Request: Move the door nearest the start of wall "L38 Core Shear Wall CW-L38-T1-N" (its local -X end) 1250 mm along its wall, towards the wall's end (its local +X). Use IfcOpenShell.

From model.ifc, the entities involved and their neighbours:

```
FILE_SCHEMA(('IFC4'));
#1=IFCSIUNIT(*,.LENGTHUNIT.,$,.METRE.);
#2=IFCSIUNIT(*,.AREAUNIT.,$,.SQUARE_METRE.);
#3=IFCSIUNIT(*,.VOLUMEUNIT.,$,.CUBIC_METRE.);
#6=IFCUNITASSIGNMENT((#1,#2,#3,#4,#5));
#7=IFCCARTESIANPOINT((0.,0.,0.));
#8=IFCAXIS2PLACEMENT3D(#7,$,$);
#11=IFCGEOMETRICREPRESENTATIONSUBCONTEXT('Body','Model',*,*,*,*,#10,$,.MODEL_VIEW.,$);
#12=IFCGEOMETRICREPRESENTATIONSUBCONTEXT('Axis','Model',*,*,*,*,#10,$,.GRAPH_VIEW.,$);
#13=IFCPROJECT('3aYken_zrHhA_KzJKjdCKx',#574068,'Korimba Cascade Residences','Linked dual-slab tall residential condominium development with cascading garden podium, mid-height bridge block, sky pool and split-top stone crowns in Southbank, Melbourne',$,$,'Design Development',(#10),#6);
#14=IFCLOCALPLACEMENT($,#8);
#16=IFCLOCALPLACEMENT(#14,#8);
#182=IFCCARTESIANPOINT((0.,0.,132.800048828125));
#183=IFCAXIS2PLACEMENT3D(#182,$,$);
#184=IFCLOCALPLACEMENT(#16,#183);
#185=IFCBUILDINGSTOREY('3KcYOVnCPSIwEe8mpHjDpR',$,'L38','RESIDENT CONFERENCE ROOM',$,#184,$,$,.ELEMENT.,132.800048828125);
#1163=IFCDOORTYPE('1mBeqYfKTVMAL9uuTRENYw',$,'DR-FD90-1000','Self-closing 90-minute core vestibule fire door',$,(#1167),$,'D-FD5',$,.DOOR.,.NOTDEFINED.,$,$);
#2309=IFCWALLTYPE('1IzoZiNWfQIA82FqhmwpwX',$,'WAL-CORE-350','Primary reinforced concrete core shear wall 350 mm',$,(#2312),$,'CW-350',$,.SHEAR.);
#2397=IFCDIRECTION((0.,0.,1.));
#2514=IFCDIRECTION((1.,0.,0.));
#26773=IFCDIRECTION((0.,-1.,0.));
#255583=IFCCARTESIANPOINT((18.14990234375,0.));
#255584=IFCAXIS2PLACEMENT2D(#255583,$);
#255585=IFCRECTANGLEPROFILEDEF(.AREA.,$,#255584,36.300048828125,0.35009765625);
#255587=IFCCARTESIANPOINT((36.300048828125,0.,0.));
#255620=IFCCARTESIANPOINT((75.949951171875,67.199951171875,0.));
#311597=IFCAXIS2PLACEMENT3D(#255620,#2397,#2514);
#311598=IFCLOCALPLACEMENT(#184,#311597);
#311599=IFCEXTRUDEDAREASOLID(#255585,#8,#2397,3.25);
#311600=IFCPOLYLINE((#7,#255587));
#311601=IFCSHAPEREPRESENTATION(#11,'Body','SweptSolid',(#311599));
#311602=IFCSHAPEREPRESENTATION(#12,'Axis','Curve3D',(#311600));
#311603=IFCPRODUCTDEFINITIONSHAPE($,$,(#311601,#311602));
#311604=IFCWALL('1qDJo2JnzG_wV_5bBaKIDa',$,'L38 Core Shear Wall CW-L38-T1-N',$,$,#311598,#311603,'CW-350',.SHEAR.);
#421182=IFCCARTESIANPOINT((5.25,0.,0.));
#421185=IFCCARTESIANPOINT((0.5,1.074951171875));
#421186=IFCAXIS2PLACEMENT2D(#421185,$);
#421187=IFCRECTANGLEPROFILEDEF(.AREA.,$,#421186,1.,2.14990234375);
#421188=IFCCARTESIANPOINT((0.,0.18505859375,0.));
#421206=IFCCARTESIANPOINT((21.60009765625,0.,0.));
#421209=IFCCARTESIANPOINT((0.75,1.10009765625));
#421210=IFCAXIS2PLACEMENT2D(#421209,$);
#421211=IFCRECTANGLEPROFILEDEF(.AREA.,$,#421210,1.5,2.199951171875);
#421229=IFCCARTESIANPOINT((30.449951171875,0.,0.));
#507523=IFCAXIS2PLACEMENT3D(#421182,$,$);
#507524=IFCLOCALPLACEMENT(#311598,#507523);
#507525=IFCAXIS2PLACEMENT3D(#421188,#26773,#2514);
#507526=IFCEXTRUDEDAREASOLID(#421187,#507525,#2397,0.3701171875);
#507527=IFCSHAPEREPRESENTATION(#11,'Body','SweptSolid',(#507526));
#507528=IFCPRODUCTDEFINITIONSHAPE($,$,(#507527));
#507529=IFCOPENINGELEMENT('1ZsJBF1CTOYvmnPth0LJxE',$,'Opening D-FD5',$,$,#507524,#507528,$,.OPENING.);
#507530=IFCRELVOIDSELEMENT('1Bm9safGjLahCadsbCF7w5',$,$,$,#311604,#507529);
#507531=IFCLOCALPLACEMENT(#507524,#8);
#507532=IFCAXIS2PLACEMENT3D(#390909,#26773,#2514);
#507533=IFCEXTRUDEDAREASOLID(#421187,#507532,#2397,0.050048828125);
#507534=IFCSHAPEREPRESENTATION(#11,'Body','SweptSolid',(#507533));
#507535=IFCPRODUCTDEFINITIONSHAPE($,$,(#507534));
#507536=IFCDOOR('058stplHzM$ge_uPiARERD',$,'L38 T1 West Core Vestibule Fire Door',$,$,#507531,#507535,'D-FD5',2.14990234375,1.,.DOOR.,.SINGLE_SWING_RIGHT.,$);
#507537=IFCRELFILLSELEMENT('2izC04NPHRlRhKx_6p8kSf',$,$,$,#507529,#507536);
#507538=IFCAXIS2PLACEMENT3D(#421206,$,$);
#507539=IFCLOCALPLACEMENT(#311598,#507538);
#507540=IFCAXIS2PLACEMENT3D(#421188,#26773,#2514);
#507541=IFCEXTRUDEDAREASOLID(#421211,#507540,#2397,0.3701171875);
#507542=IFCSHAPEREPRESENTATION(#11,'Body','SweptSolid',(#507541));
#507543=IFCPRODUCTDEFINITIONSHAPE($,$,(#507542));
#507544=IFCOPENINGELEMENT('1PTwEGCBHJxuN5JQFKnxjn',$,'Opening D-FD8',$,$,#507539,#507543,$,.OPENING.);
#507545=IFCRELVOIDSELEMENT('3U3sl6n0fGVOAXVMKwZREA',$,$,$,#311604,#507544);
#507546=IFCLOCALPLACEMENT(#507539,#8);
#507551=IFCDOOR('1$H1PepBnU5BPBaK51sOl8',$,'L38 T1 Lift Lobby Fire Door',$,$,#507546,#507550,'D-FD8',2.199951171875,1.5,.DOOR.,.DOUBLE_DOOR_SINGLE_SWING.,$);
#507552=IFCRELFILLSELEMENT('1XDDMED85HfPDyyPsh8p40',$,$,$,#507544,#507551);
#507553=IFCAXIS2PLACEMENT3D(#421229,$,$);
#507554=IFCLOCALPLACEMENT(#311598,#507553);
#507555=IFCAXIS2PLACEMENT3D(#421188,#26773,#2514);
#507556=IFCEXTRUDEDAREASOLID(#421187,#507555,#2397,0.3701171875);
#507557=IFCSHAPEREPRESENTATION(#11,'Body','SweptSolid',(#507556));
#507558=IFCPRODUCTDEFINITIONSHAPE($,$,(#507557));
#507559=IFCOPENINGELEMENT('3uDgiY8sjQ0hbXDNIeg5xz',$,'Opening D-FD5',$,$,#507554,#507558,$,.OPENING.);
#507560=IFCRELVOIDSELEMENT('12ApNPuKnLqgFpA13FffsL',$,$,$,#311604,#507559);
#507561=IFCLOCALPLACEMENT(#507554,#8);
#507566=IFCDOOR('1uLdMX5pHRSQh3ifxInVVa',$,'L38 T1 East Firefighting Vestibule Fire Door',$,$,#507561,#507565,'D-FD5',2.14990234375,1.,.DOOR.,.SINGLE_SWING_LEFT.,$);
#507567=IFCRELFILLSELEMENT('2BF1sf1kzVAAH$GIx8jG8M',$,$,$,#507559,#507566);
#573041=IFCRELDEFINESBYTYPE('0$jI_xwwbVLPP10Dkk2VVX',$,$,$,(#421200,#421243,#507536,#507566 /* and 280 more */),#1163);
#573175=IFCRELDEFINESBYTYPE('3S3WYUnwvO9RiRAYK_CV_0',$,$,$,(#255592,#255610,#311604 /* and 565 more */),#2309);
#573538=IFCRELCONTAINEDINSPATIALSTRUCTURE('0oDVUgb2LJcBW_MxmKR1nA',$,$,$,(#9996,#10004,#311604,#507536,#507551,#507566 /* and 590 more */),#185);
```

```python
import ifcopenshell
import ifcopenshell.api.geometry
import ifcopenshell.util.placement
import ifcopenshell.util.unit

model = ifcopenshell.open("model.ifc")
unit_scale = ifcopenshell.util.unit.calculate_unit_scale(model)

door = model.by_guid("058stplHzM$ge_uPiARERD")
opening = door.FillsVoids[0].RelatingOpeningElement
wall = opening.VoidsElements[0].RelatingBuildingElement

wall_matrix = ifcopenshell.util.placement.get_local_placement(wall.ObjectPlacement)
shift = wall_matrix[:3, 0] * 1.25 / unit_scale
before = ifcopenshell.util.placement.get_local_placement(door.ObjectPlacement)[:3, 3].copy()

# The door is placed relative to its opening, so it follows when the opening moves.
matrix = ifcopenshell.util.placement.get_local_placement(opening.ObjectPlacement)
matrix[:3, 3] += shift
ifcopenshell.api.geometry.edit_object_placement(
    model, product=opening, matrix=matrix, is_si=False, should_transform_children=True
)

after = ifcopenshell.util.placement.get_local_placement(door.ObjectPlacement)[:3, 3]
print("door moved by", (after - before).round(3) + 0.0)

model.write("model-out.ifc")
```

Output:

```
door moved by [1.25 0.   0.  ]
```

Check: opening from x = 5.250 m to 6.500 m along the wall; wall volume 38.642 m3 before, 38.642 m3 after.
